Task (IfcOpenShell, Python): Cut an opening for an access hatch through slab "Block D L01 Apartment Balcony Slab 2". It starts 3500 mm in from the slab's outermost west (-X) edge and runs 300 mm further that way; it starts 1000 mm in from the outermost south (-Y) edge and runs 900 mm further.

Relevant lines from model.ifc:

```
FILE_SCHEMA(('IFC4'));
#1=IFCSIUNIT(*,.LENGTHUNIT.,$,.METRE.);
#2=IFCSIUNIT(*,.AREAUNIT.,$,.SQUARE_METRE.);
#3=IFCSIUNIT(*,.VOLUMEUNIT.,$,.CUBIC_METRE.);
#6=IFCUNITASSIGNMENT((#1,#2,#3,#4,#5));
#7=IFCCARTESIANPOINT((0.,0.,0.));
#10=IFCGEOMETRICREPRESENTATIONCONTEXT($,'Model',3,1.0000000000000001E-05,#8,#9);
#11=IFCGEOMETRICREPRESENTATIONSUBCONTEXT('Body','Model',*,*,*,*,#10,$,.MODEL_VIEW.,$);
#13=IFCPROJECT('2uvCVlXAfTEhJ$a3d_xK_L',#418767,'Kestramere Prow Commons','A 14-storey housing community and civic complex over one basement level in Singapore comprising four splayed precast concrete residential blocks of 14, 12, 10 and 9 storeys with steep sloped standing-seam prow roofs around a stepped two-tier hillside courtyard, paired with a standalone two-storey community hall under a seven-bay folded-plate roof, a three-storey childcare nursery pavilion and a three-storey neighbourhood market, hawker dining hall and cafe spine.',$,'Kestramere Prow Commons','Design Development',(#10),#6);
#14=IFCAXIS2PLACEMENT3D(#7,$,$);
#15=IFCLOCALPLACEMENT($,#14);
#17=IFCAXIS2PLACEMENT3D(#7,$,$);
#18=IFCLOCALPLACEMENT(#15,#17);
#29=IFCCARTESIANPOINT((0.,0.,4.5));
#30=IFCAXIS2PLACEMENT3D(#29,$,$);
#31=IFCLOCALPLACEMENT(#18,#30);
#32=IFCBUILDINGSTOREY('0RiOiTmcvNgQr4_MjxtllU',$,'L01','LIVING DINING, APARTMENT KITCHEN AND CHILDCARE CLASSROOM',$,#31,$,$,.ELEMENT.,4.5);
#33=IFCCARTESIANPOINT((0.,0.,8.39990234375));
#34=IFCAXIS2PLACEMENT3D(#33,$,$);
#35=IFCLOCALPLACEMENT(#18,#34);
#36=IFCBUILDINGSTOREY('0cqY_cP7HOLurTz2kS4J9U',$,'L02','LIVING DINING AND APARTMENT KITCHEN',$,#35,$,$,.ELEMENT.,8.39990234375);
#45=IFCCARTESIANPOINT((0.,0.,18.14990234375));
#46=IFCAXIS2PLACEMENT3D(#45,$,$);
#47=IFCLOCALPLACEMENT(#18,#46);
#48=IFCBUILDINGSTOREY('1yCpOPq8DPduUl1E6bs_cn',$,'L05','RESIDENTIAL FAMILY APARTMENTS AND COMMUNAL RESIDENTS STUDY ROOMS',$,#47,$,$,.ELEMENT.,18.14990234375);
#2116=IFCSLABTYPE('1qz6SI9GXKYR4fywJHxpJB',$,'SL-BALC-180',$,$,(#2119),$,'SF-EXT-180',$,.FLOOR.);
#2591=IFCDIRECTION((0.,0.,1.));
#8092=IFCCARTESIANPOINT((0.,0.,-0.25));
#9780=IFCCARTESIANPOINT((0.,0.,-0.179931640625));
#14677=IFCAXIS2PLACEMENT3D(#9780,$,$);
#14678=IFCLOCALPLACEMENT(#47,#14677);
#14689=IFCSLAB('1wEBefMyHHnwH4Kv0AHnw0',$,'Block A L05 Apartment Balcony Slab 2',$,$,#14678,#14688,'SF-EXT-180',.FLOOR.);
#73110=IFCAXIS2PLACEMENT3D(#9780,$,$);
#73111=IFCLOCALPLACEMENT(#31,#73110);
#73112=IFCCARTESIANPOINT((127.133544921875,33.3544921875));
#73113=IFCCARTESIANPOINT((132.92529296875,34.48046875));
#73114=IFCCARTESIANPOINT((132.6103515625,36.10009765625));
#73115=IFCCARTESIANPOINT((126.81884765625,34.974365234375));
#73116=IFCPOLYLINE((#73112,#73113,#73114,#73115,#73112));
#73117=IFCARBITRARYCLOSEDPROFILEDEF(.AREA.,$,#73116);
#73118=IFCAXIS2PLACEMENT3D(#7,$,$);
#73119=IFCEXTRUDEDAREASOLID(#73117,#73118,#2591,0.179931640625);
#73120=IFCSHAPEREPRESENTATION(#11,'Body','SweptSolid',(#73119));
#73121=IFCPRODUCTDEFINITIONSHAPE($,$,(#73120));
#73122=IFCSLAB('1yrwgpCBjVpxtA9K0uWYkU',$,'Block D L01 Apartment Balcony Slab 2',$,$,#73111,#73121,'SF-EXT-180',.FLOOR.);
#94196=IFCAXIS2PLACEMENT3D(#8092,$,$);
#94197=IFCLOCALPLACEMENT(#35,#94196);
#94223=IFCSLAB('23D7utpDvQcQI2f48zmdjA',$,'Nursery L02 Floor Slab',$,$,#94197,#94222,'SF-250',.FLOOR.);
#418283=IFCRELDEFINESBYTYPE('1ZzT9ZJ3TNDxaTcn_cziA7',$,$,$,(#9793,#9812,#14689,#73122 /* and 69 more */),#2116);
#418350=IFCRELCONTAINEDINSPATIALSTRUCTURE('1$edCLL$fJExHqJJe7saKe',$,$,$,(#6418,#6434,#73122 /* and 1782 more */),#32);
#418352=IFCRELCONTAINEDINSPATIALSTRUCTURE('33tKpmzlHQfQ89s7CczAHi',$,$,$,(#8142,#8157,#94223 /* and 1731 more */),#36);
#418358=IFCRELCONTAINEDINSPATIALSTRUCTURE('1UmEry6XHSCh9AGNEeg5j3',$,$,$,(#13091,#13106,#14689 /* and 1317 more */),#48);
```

```python
import numpy as np
import ifcopenshell
import ifcopenshell.api.feature
import ifcopenshell.api.geometry
import ifcopenshell.api.root
import ifcopenshell.geom
import ifcopenshell.util.placement
import ifcopenshell.util.representation
import ifcopenshell.util.shape
import ifcopenshell.util.unit

model = ifcopenshell.open("model.ifc")
unit_scale = ifcopenshell.util.unit.calculate_unit_scale(model)
settings = ifcopenshell.geom.settings()


def volume(element):
    """Net volume in cubic metres, openings subtracted."""
    shape = ifcopenshell.geom.create_shape(settings, element)
    return ifcopenshell.util.shape.get_volume(shape.geometry)


slab = model.by_guid("1yrwgpCBjVpxtA9K0uWYkU")
before = volume(slab)

# Extent in the slab's own axes, in metres. The edges named are its -X and -Y sides.
slab_shape = ifcopenshell.geom.create_shape(settings, slab)
vertices = ifcopenshell.util.shape.get_vertices(slab_shape.geometry)
x_min, y_min, bottom = vertices.min(axis=0)
top = vertices[:, 2].max()

opening = ifcopenshell.api.root.create_entity(model, ifc_class="IfcOpeningElement", name="Access hatch opening", predefined_type="OPENING")
context = ifcopenshell.util.representation.get_context(model, "Model", "Body", "MODEL_VIEW")
width, depth = 0.3, 0.9
outline = [(0.0, 0.0), (width, 0.0), (width, depth), (0.0, depth), (0.0, 0.0)]
# Overshoot both faces by 50 mm so the cut is clean.
shape = ifcopenshell.api.geometry.add_slab_representation(
    model, context=context, depth=top - bottom + 0.1, polyline=outline
)
ifcopenshell.api.geometry.assign_representation(model, product=opening, representation=shape)

matrix = ifcopenshell.util.placement.get_local_placement(slab.ObjectPlacement)
matrix[:, 3] = matrix @ np.append(np.array([x_min + 3.5, y_min + 1, bottom - 0.05]) / unit_scale, 1.0)
ifcopenshell.api.geometry.edit_object_placement(model, product=opening, matrix=matrix, is_si=False)
ifcopenshell.api.feature.add_feature(model, feature=opening, element=slab)

after = volume(slab)

print(f"slab volume {before:.3f} -> {after:.3f} m3")

model.write("model-out.ifc")
```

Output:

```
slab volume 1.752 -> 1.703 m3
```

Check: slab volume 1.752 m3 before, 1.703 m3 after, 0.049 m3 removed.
